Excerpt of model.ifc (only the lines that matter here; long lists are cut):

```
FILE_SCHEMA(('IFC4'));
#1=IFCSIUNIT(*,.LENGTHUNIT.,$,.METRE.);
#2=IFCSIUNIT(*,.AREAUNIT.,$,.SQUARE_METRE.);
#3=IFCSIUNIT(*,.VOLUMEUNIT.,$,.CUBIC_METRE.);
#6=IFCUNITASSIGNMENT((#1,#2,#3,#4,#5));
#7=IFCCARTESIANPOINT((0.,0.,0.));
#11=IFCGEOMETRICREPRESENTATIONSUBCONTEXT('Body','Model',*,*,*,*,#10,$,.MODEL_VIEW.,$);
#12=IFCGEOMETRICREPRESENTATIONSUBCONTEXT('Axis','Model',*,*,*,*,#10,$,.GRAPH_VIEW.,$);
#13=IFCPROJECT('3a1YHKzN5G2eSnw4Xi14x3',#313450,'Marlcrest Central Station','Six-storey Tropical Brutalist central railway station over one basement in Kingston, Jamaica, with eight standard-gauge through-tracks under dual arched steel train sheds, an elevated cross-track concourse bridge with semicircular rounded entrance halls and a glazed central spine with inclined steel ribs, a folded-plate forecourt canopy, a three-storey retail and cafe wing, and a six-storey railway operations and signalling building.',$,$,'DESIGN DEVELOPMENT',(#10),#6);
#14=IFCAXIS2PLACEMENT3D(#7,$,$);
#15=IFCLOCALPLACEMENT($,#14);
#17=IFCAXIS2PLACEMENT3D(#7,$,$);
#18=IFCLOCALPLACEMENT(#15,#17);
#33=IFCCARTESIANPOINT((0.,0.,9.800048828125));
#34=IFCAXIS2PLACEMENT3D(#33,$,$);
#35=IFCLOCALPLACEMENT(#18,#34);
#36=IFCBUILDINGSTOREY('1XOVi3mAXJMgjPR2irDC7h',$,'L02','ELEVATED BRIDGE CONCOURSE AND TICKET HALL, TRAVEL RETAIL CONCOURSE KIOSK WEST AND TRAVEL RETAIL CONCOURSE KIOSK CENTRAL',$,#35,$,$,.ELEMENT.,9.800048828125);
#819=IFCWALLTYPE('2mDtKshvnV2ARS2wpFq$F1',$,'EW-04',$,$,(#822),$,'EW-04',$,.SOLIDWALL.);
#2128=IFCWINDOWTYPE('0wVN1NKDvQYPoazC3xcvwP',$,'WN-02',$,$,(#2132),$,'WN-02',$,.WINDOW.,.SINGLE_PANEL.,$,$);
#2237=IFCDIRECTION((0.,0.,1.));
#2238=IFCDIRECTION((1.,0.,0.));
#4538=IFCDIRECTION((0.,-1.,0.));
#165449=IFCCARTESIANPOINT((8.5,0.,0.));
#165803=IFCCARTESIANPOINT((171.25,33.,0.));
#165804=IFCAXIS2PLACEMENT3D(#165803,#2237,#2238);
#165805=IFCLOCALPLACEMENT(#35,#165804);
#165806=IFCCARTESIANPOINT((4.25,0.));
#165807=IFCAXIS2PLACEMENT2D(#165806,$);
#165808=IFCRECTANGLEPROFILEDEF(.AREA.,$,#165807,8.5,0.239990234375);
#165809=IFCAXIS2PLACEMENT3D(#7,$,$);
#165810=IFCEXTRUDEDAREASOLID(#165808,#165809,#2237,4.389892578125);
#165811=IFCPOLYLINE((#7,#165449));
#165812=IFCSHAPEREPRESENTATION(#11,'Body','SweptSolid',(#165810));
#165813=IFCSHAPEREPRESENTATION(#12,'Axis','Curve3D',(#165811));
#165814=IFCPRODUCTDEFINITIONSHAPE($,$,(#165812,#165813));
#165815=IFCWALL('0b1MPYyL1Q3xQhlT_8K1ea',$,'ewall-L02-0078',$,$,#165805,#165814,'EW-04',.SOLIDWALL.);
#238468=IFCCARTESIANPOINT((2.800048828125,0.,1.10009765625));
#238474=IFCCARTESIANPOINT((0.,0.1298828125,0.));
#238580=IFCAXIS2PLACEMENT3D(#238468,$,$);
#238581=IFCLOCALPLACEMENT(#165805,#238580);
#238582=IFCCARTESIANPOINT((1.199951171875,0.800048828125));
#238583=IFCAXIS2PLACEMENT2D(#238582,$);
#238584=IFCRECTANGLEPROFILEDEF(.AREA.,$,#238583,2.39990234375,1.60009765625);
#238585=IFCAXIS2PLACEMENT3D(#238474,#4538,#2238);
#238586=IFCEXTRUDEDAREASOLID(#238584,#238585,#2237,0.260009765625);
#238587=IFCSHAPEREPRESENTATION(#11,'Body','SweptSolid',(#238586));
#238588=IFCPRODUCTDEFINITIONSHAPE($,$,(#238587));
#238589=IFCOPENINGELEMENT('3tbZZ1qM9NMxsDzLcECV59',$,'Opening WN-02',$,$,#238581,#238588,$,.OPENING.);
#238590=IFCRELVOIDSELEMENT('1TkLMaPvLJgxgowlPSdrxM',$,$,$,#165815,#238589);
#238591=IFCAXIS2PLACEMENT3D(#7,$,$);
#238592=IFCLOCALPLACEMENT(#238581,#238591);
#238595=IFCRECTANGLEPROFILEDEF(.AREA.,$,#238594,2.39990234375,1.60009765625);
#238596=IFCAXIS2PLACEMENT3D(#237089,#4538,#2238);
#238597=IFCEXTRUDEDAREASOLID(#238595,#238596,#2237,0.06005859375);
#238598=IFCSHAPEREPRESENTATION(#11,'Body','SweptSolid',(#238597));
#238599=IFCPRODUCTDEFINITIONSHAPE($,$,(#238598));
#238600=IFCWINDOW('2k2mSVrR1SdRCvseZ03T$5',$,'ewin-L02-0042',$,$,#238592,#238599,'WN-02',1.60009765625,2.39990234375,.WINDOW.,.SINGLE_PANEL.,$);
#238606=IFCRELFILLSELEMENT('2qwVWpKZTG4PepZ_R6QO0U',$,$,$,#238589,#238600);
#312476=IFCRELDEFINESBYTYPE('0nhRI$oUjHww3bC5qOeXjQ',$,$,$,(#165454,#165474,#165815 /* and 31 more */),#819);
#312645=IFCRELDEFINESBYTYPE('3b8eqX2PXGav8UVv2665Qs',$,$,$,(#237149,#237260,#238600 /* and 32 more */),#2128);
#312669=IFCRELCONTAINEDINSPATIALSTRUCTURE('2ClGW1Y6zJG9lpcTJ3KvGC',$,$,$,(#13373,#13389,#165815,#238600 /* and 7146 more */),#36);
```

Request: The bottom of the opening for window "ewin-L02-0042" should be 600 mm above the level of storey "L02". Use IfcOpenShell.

```python
import numpy as np
import ifcopenshell
import ifcopenshell.api.geometry
import ifcopenshell.geom
import ifcopenshell.util.element
import ifcopenshell.util.placement
import ifcopenshell.util.shape
import ifcopenshell.util.unit

model = ifcopenshell.open("model.ifc")
unit_scale = ifcopenshell.util.unit.calculate_unit_scale(model)

window = model.by_guid("2k2mSVrR1SdRCvseZ03T$5")
opening = window.FillsVoids[0].RelatingOpeningElement
storey = ifcopenshell.util.element.get_container(window, ifc_class="IfcBuildingStorey")
level = ifcopenshell.util.placement.get_local_placement(storey.ObjectPlacement)[2, 3]

# The opening's origin need not be at the sill, so measure its lowest point.
shape = ifcopenshell.geom.create_shape(ifcopenshell.geom.settings(), opening)
bottom = ifcopenshell.util.shape.get_shape_bottom_elevation(shape, shape.geometry) / unit_scale
dz = level + 0.6 - bottom

shift = np.array([0.0, 0.0, dz])
# The window is placed relative to its opening, so it follows when the opening moves.
matrix = ifcopenshell.util.placement.get_local_placement(opening.ObjectPlacement)
matrix[:3, 3] += shift
ifcopenshell.api.geometry.edit_object_placement(
    model, product=opening, matrix=matrix, is_si=False, should_transform_children=True
)

print(f"moved by {dz * unit_scale:+.3f} m")

model.write("model_edited.ifc")
```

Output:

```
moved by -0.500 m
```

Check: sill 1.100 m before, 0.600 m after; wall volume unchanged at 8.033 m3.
